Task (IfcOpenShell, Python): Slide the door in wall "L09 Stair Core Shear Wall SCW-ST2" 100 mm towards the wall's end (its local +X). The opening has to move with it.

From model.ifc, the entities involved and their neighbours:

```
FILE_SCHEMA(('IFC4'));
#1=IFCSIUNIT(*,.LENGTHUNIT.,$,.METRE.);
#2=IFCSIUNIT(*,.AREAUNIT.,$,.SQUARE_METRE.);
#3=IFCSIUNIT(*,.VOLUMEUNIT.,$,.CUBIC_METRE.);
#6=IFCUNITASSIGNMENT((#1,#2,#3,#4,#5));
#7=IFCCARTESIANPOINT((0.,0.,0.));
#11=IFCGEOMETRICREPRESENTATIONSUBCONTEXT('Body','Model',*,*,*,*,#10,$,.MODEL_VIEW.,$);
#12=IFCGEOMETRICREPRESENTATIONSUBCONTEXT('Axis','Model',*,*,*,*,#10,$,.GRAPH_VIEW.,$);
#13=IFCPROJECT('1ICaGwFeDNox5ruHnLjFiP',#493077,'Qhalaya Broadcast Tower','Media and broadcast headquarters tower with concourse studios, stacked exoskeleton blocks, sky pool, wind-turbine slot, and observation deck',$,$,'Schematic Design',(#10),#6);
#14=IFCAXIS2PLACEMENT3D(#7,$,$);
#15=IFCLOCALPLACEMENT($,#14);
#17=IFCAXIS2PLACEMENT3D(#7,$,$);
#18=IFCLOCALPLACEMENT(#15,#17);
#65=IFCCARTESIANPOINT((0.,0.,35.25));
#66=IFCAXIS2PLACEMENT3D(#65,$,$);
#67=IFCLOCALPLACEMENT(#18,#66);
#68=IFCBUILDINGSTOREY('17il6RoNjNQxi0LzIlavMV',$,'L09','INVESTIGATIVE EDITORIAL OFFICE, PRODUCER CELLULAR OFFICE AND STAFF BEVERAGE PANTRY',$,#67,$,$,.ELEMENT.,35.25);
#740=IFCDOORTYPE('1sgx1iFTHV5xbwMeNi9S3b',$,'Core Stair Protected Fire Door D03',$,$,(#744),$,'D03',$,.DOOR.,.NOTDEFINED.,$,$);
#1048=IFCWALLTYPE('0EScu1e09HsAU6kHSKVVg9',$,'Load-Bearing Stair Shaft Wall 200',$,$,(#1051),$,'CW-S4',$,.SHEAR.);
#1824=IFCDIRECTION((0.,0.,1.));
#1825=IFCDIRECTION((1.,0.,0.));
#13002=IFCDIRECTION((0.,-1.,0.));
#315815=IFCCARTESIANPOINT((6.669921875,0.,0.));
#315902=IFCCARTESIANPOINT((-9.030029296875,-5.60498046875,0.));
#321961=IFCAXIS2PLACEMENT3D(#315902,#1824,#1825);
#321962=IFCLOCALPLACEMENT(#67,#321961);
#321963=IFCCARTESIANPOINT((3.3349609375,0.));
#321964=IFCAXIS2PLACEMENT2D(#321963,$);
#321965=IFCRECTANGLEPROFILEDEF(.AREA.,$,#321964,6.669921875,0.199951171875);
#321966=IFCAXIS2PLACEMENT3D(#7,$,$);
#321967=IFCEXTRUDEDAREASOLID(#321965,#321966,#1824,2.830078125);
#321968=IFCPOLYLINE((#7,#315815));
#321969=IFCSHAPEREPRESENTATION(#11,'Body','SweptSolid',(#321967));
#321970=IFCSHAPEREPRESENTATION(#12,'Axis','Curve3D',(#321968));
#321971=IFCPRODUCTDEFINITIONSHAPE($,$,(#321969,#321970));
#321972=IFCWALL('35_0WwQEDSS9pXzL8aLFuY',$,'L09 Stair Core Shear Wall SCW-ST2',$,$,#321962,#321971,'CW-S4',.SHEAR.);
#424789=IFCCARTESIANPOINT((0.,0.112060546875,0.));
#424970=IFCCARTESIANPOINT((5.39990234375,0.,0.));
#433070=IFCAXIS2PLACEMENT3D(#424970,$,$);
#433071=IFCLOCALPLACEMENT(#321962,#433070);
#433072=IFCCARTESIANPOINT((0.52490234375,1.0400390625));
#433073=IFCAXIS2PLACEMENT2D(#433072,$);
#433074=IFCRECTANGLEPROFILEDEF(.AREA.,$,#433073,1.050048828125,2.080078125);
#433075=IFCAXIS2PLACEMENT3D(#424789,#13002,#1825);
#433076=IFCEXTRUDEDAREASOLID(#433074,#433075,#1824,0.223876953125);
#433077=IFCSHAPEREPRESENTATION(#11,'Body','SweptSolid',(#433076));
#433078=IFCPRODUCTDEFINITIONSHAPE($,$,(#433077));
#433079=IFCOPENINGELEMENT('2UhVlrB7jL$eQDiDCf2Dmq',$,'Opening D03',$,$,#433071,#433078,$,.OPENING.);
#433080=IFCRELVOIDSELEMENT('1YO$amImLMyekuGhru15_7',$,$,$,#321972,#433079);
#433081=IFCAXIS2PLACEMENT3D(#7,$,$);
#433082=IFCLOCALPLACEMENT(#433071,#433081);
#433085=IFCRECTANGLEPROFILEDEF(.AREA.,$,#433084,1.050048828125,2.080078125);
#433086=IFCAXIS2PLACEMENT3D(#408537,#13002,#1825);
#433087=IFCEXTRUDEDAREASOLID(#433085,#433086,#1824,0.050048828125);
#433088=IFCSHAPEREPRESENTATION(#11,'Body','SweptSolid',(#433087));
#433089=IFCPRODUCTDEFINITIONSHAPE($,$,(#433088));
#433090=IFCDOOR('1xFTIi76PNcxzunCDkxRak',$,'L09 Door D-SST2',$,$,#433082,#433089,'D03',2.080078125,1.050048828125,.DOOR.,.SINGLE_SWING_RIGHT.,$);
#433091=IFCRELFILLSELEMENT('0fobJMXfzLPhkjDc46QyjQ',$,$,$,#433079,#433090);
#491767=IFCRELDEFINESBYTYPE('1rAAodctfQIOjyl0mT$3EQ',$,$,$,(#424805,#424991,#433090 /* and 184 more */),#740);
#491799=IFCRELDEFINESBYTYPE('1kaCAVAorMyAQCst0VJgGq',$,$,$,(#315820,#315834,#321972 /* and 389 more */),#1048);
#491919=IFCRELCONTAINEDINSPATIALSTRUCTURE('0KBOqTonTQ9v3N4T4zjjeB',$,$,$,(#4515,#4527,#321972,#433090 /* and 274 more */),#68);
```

```python
import ifcopenshell
import ifcopenshell.api.geometry
import ifcopenshell.util.placement
import ifcopenshell.util.unit

model = ifcopenshell.open("model.ifc")
unit_scale = ifcopenshell.util.unit.calculate_unit_scale(model)

door = model.by_guid("1xFTIi76PNcxzunCDkxRak")
opening = door.FillsVoids[0].RelatingOpeningElement
wall = opening.VoidsElements[0].RelatingBuildingElement

wall_matrix = ifcopenshell.util.placement.get_local_placement(wall.ObjectPlacement)
shift = wall_matrix[:3, 0] * 0.1 / unit_scale
before = ifcopenshell.util.placement.get_local_placement(door.ObjectPlacement)[:3, 3].copy()

# The door is placed relative to its opening, so it follows when the opening moves.
matrix = ifcopenshell.util.placement.get_local_placement(opening.ObjectPlacement)
matrix[:3, 3] += shift
ifcopenshell.api.geometry.edit_object_placement(
    model, product=opening, matrix=matrix, is_si=False, should_transform_children=True
)

after = ifcopenshell.util.placement.get_local_placement(door.ObjectPlacement)[:3, 3]
print("door moved by", (after - before).round(3) + 0.0)

model.write("model_rev.ifc")
```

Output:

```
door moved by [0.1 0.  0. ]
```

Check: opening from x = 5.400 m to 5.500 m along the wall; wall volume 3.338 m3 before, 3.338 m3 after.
